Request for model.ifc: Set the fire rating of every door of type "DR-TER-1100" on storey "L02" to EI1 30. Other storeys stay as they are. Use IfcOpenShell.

First a look at what the model holds.

```python
import ifcopenshell
import ifcopenshell.util.element

model = ifcopenshell.open("model.ifc")
print(model.schema)
storey = next(s for s in model.by_type("IfcBuildingStorey") if s.Name == "L02")
doors = [e for e in ifcopenshell.util.element.get_decomposition(storey) if e.is_a("IfcDoor")]
seen = {}
for e in doors:
    element_type = ifcopenshell.util.element.get_type(e)
    key = (element_type.Name if element_type != e and element_type else None, ifcopenshell.util.element.get_pset(e, "Pset_DoorCommon", "FireRating"))
    seen[key] = seen.get(key, 0) + 1
for (name, value), count in sorted(seen.items(), key=str):
    print(count, "x", name, "|", value)
```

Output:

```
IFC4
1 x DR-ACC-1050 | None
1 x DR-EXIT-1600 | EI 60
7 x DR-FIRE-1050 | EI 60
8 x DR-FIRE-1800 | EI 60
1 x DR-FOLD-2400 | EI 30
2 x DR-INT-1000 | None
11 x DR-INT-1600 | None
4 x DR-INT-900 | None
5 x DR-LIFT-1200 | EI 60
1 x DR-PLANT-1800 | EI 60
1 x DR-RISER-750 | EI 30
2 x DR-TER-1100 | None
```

```python
import ifcopenshell
import ifcopenshell.api.pset
import ifcopenshell.util.element

model = ifcopenshell.open("model.ifc")

storey = next(s for s in model.by_type("IfcBuildingStorey") if s.Name == "L02")
doors = [e for e in ifcopenshell.util.element.get_decomposition(storey) if e.is_a("IfcDoor")]

count = 0
for e in doors:
    element_type = ifcopenshell.util.element.get_type(e)
    if element_type in (None, e) or element_type.Name != "DR-TER-1100":
        continue
    # add_pset returns the element's existing set when there is one.
    pset = ifcopenshell.api.pset.add_pset(model, product=e, name="Pset_DoorCommon")
    ifcopenshell.api.pset.edit_pset(model, pset=pset, properties={"FireRating": "EI1 30"})
    count += 1

print(count, "doors updated")

model.write("model_updated.ifc")
```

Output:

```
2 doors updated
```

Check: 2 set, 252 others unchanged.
